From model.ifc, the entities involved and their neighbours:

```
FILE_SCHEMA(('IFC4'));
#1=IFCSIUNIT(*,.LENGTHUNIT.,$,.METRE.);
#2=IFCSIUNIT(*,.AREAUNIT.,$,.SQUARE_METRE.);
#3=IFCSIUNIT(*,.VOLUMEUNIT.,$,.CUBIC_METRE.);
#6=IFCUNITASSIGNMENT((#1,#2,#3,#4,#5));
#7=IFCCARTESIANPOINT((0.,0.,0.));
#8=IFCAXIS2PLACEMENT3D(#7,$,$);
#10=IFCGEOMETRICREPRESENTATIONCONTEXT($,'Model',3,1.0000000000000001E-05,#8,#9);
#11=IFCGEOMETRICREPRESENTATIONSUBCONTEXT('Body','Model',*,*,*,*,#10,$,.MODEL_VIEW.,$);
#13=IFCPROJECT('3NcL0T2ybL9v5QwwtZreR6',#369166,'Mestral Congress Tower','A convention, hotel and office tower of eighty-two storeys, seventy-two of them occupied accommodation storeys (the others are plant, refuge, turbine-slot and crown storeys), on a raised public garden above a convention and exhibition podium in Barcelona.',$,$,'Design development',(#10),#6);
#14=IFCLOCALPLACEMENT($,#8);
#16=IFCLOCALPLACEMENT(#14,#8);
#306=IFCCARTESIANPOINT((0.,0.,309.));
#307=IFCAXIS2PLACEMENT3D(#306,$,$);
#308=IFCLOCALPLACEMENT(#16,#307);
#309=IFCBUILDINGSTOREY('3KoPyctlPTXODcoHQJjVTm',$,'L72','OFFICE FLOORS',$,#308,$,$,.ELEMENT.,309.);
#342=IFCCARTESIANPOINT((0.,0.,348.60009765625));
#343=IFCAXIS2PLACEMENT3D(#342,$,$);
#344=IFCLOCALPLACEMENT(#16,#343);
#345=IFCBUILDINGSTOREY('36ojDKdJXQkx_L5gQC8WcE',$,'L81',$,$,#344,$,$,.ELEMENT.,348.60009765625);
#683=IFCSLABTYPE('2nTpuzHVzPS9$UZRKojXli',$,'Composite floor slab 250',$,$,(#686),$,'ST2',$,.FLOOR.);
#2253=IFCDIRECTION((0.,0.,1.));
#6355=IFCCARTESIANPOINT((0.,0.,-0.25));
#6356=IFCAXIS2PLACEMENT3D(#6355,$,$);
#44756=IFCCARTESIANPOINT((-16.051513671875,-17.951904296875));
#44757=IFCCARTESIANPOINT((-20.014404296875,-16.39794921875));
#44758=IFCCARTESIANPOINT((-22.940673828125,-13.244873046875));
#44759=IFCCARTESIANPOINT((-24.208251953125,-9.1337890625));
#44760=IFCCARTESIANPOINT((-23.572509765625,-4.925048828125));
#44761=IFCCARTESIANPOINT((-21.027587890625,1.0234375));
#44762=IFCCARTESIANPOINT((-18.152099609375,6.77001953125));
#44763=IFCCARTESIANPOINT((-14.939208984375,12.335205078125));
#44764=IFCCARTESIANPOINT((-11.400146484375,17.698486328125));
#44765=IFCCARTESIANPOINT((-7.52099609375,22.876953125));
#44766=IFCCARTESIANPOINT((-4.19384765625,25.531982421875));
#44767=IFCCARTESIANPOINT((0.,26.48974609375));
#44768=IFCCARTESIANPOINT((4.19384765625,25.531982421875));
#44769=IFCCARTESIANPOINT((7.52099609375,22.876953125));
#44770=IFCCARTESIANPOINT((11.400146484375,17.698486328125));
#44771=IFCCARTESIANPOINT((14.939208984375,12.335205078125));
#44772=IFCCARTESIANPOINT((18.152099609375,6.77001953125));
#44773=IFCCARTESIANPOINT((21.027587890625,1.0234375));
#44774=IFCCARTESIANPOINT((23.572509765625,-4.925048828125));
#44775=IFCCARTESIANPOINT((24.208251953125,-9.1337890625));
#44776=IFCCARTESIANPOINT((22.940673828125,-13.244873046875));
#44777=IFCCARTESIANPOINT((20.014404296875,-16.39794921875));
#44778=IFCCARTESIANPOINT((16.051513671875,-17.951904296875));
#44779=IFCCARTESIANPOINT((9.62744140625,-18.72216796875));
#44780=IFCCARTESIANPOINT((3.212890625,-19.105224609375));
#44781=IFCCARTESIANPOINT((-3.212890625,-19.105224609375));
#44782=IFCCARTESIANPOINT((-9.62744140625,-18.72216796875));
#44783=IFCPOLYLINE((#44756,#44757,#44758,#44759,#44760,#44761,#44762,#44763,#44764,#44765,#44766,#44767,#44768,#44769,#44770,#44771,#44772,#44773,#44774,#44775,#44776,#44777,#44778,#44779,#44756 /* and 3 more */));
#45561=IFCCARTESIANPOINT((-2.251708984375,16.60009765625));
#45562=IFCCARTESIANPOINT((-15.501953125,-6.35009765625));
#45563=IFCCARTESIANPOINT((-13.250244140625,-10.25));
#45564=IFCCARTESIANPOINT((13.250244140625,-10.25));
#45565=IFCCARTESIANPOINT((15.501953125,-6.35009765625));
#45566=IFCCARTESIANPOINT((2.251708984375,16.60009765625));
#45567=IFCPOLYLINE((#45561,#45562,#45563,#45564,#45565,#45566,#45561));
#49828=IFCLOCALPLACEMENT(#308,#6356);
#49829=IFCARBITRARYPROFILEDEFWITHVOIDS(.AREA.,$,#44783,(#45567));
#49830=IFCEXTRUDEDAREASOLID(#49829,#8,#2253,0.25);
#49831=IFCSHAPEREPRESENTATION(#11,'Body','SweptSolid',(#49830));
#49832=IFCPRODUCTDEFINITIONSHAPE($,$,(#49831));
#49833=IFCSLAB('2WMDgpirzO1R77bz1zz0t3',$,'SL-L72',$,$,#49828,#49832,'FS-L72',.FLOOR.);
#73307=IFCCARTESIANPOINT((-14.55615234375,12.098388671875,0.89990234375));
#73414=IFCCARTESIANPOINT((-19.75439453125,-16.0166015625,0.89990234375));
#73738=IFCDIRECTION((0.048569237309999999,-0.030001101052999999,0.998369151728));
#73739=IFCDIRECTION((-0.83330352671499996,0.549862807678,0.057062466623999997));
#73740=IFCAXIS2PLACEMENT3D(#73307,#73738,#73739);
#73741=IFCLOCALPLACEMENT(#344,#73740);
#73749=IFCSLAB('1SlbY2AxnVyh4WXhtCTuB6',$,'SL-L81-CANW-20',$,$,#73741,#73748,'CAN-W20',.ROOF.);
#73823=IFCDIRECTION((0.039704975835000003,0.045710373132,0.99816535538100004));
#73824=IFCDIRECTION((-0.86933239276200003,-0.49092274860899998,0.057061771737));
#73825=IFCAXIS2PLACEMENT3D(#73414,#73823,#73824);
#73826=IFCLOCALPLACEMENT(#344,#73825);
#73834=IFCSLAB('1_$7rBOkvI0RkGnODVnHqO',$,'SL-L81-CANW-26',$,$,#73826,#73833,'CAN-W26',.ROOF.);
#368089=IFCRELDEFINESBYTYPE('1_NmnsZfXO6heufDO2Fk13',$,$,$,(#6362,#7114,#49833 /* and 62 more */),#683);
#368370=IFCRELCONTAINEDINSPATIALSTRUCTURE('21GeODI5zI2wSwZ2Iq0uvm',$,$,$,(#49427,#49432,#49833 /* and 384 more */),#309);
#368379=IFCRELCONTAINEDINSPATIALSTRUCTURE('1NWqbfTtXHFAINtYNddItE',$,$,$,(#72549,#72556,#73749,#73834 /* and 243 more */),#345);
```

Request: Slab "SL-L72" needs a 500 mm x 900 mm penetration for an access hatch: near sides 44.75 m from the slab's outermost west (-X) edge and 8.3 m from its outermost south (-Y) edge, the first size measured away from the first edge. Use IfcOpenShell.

```python
import numpy as np
import ifcopenshell
import ifcopenshell.api.feature
import ifcopenshell.api.geometry
import ifcopenshell.api.root
import ifcopenshell.geom
import ifcopenshell.util.placement
import ifcopenshell.util.representation
import ifcopenshell.util.shape
import ifcopenshell.util.unit

model = ifcopenshell.open("model.ifc")
unit_scale = ifcopenshell.util.unit.calculate_unit_scale(model)
settings = ifcopenshell.geom.settings()


def volume(element):
    """Net volume in cubic metres, openings subtracted."""
    shape = ifcopenshell.geom.create_shape(settings, element)
    return ifcopenshell.util.shape.get_volume(shape.geometry)


slab = model.by_guid("2WMDgpirzO1R77bz1zz0t3")
before = volume(slab)

# Extent in the slab's own axes, in metres. The edges named are its -X and -Y sides.
slab_shape = ifcopenshell.geom.create_shape(settings, slab)
vertices = ifcopenshell.util.shape.get_vertices(slab_shape.geometry)
x_min, y_min, bottom = vertices.min(axis=0)
top = vertices[:, 2].max()

opening = ifcopenshell.api.root.create_entity(model, ifc_class="IfcOpeningElement", name="Access hatch opening", predefined_type="OPENING")
context = ifcopenshell.util.representation.get_context(model, "Model", "Body", "MODEL_VIEW")
width, depth = 0.5, 0.9
outline = [(0.0, 0.0), (width, 0.0), (width, depth), (0.0, depth), (0.0, 0.0)]
# Overshoot both faces by 50 mm so the cut is clean.
shape = ifcopenshell.api.geometry.add_slab_representation(
    model, context=context, depth=top - bottom + 0.1, polyline=outline
)
ifcopenshell.api.geometry.assign_representation(model, product=opening, representation=shape)

matrix = ifcopenshell.util.placement.get_local_placement(slab.ObjectPlacement)
matrix[:, 3] = matrix @ np.append(np.array([x_min + 44.75, y_min + 8.3, bottom - 0.05]) / unit_scale, 1.0)
ifcopenshell.api.geometry.edit_object_placement(model, product=opening, matrix=matrix, is_si=False)
ifcopenshell.api.feature.add_feature(model, feature=opening, element=slab)

after = volume(slab)

print(f"slab volume {before:.3f} -> {after:.3f} m3")

model.write("model_rev.ifc")
```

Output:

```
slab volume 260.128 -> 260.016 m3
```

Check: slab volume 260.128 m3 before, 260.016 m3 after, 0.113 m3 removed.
